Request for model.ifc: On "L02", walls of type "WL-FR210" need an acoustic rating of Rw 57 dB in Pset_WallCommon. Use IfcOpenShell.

First a look at what the model holds.

```python
import ifcopenshell
import ifcopenshell.util.element

model = ifcopenshell.open("model.ifc")
print(model.schema)
storey = next(s for s in model.by_type("IfcBuildingStorey") if s.Name == "L02")
walls = [e for e in ifcopenshell.util.element.get_decomposition(storey) if e.is_a("IfcWall")]
seen = {}
for e in walls:
    element_type = ifcopenshell.util.element.get_type(e)
    key = (element_type.Name if element_type != e and element_type else None, ifcopenshell.util.element.get_pset(e, "Pset_WallCommon", "AcousticRating"))
    seen[key] = seen.get(key, 0) + 1
for (name, value), count in sorted(seen.items(), key=str):
    print(count, "x", name, "|", value)
```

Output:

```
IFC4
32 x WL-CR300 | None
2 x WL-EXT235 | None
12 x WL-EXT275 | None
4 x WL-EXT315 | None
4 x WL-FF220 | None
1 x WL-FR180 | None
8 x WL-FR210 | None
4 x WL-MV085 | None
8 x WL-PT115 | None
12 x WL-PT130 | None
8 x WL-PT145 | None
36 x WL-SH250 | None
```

```python
import ifcopenshell
import ifcopenshell.api.pset
import ifcopenshell.util.element

model = ifcopenshell.open("model.ifc")

storey = next(s for s in model.by_type("IfcBuildingStorey") if s.Name == "L02")
walls = [e for e in ifcopenshell.util.element.get_decomposition(storey) if e.is_a("IfcWall")]

count = 0
for e in walls:
    element_type = ifcopenshell.util.element.get_type(e)
    if element_type in (None, e) or element_type.Name != "WL-FR210":
        continue
    # add_pset returns the element's existing set when there is one.
    pset = ifcopenshell.api.pset.add_pset(model, product=e, name="Pset_WallCommon")
    ifcopenshell.api.pset.edit_pset(model, pset=pset, properties={"AcousticRating": "Rw 57 dB"})
    count += 1

print(count, "walls updated")

model.write("model_updated.ifc")
```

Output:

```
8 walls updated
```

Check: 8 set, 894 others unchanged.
